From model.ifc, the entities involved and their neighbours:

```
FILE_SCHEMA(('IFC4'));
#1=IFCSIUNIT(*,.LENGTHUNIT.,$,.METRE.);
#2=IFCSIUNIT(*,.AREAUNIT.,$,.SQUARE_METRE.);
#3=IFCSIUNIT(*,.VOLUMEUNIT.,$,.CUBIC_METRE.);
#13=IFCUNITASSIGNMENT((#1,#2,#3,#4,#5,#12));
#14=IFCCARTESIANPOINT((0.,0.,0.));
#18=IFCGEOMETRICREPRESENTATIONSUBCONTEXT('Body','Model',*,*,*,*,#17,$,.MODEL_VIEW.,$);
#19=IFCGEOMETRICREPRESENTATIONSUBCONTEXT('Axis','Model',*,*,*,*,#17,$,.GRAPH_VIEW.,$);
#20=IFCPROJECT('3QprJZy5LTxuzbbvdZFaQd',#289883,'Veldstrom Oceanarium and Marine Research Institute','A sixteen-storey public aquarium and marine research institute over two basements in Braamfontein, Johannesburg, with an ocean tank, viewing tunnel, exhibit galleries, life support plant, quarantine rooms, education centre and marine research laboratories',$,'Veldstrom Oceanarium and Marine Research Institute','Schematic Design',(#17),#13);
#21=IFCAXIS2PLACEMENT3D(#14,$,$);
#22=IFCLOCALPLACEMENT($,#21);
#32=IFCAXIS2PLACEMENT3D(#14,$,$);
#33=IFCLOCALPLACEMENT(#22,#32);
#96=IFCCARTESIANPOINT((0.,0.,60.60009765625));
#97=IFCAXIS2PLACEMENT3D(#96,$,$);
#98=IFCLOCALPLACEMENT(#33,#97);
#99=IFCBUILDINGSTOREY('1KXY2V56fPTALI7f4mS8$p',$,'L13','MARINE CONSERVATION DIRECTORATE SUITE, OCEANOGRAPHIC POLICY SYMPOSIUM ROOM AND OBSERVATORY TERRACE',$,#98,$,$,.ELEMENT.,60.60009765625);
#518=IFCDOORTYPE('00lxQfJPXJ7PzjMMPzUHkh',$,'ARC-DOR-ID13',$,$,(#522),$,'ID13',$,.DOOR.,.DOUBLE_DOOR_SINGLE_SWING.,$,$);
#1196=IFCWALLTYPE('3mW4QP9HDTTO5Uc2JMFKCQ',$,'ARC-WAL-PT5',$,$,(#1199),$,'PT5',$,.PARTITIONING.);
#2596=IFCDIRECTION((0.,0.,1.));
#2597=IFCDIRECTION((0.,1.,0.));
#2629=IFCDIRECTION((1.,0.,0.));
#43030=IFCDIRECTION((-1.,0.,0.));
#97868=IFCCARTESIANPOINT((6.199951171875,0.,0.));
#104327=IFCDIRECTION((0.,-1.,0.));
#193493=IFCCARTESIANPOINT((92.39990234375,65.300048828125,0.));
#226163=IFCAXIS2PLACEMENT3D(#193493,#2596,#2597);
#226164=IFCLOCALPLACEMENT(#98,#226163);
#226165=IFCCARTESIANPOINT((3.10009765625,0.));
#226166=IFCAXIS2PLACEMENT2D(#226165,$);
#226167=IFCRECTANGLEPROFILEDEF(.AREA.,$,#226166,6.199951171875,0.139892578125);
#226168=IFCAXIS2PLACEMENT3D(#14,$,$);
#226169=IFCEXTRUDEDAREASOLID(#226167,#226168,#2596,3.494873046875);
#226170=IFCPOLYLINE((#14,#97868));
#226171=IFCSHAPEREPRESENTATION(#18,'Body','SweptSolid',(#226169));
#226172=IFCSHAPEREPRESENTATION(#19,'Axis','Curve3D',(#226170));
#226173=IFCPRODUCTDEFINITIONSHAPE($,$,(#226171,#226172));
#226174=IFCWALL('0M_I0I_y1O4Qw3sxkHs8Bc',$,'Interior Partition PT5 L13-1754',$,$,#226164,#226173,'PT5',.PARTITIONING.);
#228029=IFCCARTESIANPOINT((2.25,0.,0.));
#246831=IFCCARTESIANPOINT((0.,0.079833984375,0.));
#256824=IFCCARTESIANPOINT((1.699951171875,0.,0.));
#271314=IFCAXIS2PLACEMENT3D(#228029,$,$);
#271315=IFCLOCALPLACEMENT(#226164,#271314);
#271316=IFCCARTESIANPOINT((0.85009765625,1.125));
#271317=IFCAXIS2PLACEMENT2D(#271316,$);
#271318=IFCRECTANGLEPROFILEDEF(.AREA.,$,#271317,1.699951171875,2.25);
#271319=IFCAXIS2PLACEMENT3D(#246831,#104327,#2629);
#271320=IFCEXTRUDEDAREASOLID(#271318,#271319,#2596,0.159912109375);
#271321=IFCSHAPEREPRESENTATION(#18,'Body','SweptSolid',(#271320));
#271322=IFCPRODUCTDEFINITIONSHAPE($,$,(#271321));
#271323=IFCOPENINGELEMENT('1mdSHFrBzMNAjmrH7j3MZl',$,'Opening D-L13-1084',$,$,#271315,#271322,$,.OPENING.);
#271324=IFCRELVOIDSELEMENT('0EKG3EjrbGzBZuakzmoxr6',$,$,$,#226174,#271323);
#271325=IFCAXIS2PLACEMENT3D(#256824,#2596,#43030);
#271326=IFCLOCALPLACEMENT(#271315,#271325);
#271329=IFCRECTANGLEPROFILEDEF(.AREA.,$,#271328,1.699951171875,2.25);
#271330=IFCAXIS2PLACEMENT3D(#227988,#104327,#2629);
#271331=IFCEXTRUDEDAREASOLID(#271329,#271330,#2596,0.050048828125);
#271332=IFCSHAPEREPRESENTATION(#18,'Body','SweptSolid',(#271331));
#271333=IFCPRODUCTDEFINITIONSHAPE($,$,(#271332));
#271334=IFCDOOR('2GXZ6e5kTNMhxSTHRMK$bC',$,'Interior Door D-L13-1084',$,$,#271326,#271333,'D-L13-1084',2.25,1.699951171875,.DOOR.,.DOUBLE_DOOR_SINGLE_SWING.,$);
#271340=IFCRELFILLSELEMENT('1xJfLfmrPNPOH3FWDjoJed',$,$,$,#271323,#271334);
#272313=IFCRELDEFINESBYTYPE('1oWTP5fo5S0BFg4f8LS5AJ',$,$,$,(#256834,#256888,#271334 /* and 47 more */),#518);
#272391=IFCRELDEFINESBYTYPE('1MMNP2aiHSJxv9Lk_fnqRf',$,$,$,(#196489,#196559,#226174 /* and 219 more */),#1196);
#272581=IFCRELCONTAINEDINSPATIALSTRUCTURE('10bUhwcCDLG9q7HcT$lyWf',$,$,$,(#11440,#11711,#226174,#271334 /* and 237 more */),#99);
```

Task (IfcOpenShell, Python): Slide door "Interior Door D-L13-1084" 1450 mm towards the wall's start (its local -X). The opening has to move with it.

```python
import ifcopenshell
import ifcopenshell.api.geometry
import ifcopenshell.util.placement
import ifcopenshell.util.unit

model = ifcopenshell.open("model.ifc")
unit_scale = ifcopenshell.util.unit.calculate_unit_scale(model)

door = model.by_guid("2GXZ6e5kTNMhxSTHRMK$bC")
opening = door.FillsVoids[0].RelatingOpeningElement
wall = opening.VoidsElements[0].RelatingBuildingElement

wall_matrix = ifcopenshell.util.placement.get_local_placement(wall.ObjectPlacement)
shift = wall_matrix[:3, 0] * -1.45 / unit_scale
before = ifcopenshell.util.placement.get_local_placement(door.ObjectPlacement)[:3, 3].copy()

# The door is placed relative to its opening, so it follows when the opening moves.
matrix = ifcopenshell.util.placement.get_local_placement(opening.ObjectPlacement)
matrix[:3, 3] += shift
ifcopenshell.api.geometry.edit_object_placement(
    model, product=opening, matrix=matrix, is_si=False, should_transform_children=True
)

after = ifcopenshell.util.placement.get_local_placement(door.ObjectPlacement)[:3, 3]
print("door moved by", (after - before).round(3) + 0.0)

model.write("model_v2.ifc")
```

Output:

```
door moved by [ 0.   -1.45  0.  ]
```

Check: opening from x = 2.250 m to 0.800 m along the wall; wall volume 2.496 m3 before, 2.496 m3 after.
